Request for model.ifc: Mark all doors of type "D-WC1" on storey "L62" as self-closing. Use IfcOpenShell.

First a look at what the model holds.

```python
import ifcopenshell
import ifcopenshell.util.element

model = ifcopenshell.open("model.ifc")
print(model.schema)
storey = next(s for s in model.by_type("IfcBuildingStorey") if s.Name == "L62")
doors = [e for e in ifcopenshell.util.element.get_decomposition(storey) if e.is_a("IfcDoor")]
seen = {}
for e in doors:
    element_type = ifcopenshell.util.element.get_type(e)
    key = (element_type.Name if element_type != e and element_type else None, ifcopenshell.util.element.get_pset(e, "Pset_DoorCommon", "SelfClosing"))
    seen[key] = seen.get(key, 0) + 1
for (name, value), count in sorted(seen.items(), key=str):
    print(count, "x", name, "|", value)
```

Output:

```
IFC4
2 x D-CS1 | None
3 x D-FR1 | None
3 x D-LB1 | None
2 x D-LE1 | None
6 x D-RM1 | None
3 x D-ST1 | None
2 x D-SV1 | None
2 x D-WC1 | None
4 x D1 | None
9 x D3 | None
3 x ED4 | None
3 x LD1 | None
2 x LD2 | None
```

```python
import ifcopenshell
import ifcopenshell.api.pset
import ifcopenshell.util.element

model = ifcopenshell.open("model.ifc")

storey = next(s for s in model.by_type("IfcBuildingStorey") if s.Name == "L62")
doors = [e for e in ifcopenshell.util.element.get_decomposition(storey) if e.is_a("IfcDoor")]

count = 0
for e in doors:
    element_type = ifcopenshell.util.element.get_type(e)
    if element_type in (None, e) or element_type.Name != "D-WC1":
        continue
    found = ifcopenshell.util.element.get_pset(e, "Pset_DoorCommon", should_inherit=False)
    if found:
        pset = model.by_id(found["id"])
        if len(ifcopenshell.util.element.get_elements_by_pset(pset)) > 1:
            pset = ifcopenshell.api.pset.unshare_pset(model, products=[e], pset=pset)[0]
    else:
        pset = ifcopenshell.api.pset.add_pset(model, product=e, name="Pset_DoorCommon")
    ifcopenshell.api.pset.edit_pset(model, pset=pset, properties={"SelfClosing": True})
    count += 1

print(count, "doors updated")

model.write("model-out.ifc")
```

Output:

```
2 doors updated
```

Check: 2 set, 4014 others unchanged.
